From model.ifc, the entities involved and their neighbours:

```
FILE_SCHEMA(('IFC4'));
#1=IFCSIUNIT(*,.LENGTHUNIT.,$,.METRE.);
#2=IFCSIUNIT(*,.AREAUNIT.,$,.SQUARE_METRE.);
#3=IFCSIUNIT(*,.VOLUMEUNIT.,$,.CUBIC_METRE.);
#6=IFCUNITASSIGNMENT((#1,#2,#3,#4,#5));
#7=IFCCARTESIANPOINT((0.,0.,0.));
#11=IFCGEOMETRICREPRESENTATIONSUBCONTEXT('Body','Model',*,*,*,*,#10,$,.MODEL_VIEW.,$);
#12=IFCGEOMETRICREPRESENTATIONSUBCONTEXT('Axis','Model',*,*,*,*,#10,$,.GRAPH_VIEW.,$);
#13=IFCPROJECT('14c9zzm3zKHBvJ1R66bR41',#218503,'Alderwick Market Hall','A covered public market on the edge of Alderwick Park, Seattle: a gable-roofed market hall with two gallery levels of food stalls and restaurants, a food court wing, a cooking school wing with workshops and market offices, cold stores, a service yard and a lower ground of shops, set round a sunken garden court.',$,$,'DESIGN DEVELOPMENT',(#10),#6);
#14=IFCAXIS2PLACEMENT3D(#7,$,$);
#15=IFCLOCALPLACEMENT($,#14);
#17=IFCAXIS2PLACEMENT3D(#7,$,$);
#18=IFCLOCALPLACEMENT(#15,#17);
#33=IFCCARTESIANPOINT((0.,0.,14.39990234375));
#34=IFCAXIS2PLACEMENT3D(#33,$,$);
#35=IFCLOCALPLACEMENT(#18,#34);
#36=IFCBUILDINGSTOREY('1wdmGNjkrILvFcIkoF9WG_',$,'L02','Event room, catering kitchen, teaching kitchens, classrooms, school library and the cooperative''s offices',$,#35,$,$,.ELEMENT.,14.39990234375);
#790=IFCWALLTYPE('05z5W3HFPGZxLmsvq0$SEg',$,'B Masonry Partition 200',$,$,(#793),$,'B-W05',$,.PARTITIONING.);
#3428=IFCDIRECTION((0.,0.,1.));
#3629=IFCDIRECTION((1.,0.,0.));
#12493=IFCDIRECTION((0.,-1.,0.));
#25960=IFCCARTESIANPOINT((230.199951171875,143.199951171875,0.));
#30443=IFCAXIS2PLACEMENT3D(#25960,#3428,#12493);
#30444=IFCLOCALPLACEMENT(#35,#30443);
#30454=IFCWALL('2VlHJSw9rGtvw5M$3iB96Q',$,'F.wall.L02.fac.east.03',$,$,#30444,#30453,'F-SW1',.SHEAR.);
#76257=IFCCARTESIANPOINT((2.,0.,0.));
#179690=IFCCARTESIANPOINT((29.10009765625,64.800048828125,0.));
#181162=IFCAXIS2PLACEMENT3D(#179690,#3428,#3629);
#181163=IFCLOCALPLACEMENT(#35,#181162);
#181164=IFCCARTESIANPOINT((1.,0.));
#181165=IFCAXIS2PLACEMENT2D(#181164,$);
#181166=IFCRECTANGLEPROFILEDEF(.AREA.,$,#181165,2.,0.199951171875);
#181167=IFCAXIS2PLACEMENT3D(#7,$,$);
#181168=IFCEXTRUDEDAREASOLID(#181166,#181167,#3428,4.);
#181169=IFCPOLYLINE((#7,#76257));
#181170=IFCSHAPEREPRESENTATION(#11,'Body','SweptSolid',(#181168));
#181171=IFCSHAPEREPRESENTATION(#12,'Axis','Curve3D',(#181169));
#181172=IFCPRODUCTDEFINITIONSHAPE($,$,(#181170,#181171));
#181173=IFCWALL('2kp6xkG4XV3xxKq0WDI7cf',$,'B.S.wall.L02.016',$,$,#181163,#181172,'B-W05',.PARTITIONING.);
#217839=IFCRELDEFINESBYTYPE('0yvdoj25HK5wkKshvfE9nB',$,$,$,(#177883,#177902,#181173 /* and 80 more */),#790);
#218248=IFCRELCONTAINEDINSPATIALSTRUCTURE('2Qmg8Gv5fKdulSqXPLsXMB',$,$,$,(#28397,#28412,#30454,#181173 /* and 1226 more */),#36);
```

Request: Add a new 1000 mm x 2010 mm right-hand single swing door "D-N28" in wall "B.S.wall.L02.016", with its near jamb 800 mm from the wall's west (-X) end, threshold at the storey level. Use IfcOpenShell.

```python
import numpy as np
import ifcopenshell
import ifcopenshell.api.feature
import ifcopenshell.api.geometry
import ifcopenshell.api.root
import ifcopenshell.api.spatial
import ifcopenshell.geom
import ifcopenshell.util.element
import ifcopenshell.util.placement
import ifcopenshell.util.representation
import ifcopenshell.util.shape
import ifcopenshell.util.unit

model = ifcopenshell.open("model.ifc")
unit_scale = ifcopenshell.util.unit.calculate_unit_scale(model)
settings = ifcopenshell.geom.settings()


def volume(element):
    """Net volume in cubic metres, openings subtracted."""
    shape = ifcopenshell.geom.create_shape(settings, element)
    return ifcopenshell.util.shape.get_volume(shape.geometry)


wall = model.by_guid("2kp6xkG4XV3xxKq0WDI7cf")
storey = ifcopenshell.util.element.get_container(wall, ifc_class="IfcBuildingStorey")
context = ifcopenshell.util.representation.get_context(model, "Model", "Body", "MODEL_VIEW")
before = volume(wall)

width, height, from_end, sill = 1, 2.01, 0.8, 0.0  # metres

# The wall runs along its own X axis, and the end named is its -X end.
wall_shape = ifcopenshell.geom.create_shape(settings, wall)
x, y, z = ifcopenshell.util.shape.get_vertices(wall_shape.geometry).T
start = x.min() + from_end
face, thickness = float(y.min()), float(y.max() - y.min())
wall_matrix = ifcopenshell.util.placement.get_local_placement(wall.ObjectPlacement)
level = ifcopenshell.util.placement.get_local_placement(storey.ObjectPlacement)[2, 3]


def in_wall(x, y):
    """Placement at x, y metres in the wall's axes, at sill height."""
    matrix = wall_matrix.copy()
    matrix[:, 3] = wall_matrix @ np.array([x / unit_scale, y / unit_scale, 0.0, 1.0])
    matrix[2, 3] = level + sill / unit_scale
    return matrix


# Opening: a box that overshoots both wall faces by 50 mm.
opening = ifcopenshell.api.root.create_entity(model, ifc_class="IfcOpeningElement", predefined_type="OPENING")
box = ifcopenshell.api.geometry.add_wall_representation(
    model, context=context, length=width, height=height, thickness=thickness + 0.1
)
ifcopenshell.api.geometry.assign_representation(model, product=opening, representation=box)
ifcopenshell.api.geometry.edit_object_placement(model, product=opening, matrix=in_wall(start, face - 0.05), is_si=False)
ifcopenshell.api.feature.add_feature(model, feature=opening, element=wall)

door = ifcopenshell.api.root.create_entity(model, ifc_class="IfcDoor", name="D-N28", predefined_type="DOOR")
door.OverallWidth, door.OverallHeight = width / unit_scale, height / unit_scale
door.OperationType = "SINGLE_SWING_RIGHT"
body = ifcopenshell.api.geometry.add_door_representation(
    model,
    context=context,
    overall_width=door.OverallWidth,
    overall_height=door.OverallHeight,
    operation_type="SINGLE_SWING_RIGHT",
    lining_properties={"LiningDepth": thickness / unit_scale, "ThresholdDepth": thickness / unit_scale},
)
ifcopenshell.api.geometry.assign_representation(model, product=door, representation=body)
ifcopenshell.api.spatial.assign_container(model, products=[door], relating_structure=storey)
ifcopenshell.api.feature.add_filling(model, opening=opening, element=door)

# The lining spans the wall, so the door starts at the wall face.
ifcopenshell.api.geometry.edit_object_placement(model, product=door, matrix=in_wall(start, face), is_si=False)

after = volume(wall)

print(f"wall volume {before:.3f} -> {after:.3f} m3")

model.write("model_edited.ifc")
```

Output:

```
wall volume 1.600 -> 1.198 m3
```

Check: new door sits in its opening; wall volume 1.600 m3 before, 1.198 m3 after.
